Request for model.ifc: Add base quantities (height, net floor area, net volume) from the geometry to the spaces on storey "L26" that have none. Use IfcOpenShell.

First a look at what the model holds.

```python
import ifcopenshell
import ifcopenshell.util.element
import ifcopenshell.util.unit

model = ifcopenshell.open("model.ifc")
print(model.schema)
for unit_type in ("LENGTHUNIT", "AREAUNIT", "VOLUMEUNIT"):
    print(unit_type, ifcopenshell.util.unit.calculate_unit_scale(model, unit_type))
storey = next(s for s in model.by_type("IfcBuildingStorey") if s.Name == "L26")
spaces = [e for e in ifcopenshell.util.element.get_decomposition(storey) if e.is_a("IfcSpace")]
for e in sorted(spaces, key=lambda e: e.id()):
    print(e.id(), e.is_a(), e.Name, list(ifcopenshell.util.element.get_psets(e, qtos_only=True)), sep=" | ")
```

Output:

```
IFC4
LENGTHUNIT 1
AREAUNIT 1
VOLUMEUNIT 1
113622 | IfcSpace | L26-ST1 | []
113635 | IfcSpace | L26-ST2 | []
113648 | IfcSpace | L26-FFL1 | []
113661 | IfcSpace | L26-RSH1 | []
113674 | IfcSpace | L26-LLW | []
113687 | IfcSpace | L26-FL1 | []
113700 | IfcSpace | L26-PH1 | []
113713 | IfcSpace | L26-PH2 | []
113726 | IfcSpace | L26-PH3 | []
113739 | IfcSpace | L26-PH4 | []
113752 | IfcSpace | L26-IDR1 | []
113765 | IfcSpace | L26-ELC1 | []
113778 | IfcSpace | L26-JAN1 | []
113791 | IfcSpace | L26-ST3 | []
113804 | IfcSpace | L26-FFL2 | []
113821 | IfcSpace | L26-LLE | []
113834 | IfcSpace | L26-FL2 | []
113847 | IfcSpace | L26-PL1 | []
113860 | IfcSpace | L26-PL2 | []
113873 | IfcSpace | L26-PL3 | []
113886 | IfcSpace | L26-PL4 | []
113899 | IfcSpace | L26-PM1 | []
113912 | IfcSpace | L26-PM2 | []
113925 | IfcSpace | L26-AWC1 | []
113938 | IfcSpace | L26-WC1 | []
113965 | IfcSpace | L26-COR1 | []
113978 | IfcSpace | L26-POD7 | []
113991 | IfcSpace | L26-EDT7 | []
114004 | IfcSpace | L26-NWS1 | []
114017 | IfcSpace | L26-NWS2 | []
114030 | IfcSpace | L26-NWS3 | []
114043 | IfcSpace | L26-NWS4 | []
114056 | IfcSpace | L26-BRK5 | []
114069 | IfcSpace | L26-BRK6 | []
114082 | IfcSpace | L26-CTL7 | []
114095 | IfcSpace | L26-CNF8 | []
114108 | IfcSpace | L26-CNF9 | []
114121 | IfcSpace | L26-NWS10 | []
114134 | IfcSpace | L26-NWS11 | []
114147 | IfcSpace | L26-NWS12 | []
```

```python
import ifcopenshell
import ifcopenshell.api.pset
import ifcopenshell.geom
import ifcopenshell.util.element
import ifcopenshell.util.shape
import ifcopenshell.util.unit

model = ifcopenshell.open("model.ifc")
unit_scale = ifcopenshell.util.unit.calculate_unit_scale(model)
area_scale = ifcopenshell.util.unit.calculate_unit_scale(model, "AREAUNIT")
volume_scale = ifcopenshell.util.unit.calculate_unit_scale(model, "VOLUMEUNIT")
settings = ifcopenshell.geom.settings()

storey = next(s for s in model.by_type("IfcBuildingStorey") if s.Name == "L26")
spaces = [e for e in ifcopenshell.util.element.get_decomposition(storey) if e.is_a("IfcSpace")]

for e in sorted(spaces, key=lambda e: e.id()):
    if ifcopenshell.util.element.get_psets(e, qtos_only=True, should_inherit=False):
        continue
    # Geometry comes back in metres, in the element's own axes.
    shape = ifcopenshell.geom.create_shape(settings, e)
    values = {
        "Height": ifcopenshell.util.shape.get_z(shape.geometry) / unit_scale,
        "NetFloorArea": ifcopenshell.util.shape.get_footprint_area(shape.geometry) / area_scale,
        "NetVolume": ifcopenshell.util.shape.get_volume(shape.geometry) / volume_scale,
    }
    qto = ifcopenshell.api.pset.add_qto(model, product=e, name="Qto_SpaceBaseQuantities")
    ifcopenshell.api.pset.edit_qto(model, qto=qto, properties=values)
    print(e.id(), {k: round(v, 3) for k, v in values.items()})

model.write("model_rev.ifc")
```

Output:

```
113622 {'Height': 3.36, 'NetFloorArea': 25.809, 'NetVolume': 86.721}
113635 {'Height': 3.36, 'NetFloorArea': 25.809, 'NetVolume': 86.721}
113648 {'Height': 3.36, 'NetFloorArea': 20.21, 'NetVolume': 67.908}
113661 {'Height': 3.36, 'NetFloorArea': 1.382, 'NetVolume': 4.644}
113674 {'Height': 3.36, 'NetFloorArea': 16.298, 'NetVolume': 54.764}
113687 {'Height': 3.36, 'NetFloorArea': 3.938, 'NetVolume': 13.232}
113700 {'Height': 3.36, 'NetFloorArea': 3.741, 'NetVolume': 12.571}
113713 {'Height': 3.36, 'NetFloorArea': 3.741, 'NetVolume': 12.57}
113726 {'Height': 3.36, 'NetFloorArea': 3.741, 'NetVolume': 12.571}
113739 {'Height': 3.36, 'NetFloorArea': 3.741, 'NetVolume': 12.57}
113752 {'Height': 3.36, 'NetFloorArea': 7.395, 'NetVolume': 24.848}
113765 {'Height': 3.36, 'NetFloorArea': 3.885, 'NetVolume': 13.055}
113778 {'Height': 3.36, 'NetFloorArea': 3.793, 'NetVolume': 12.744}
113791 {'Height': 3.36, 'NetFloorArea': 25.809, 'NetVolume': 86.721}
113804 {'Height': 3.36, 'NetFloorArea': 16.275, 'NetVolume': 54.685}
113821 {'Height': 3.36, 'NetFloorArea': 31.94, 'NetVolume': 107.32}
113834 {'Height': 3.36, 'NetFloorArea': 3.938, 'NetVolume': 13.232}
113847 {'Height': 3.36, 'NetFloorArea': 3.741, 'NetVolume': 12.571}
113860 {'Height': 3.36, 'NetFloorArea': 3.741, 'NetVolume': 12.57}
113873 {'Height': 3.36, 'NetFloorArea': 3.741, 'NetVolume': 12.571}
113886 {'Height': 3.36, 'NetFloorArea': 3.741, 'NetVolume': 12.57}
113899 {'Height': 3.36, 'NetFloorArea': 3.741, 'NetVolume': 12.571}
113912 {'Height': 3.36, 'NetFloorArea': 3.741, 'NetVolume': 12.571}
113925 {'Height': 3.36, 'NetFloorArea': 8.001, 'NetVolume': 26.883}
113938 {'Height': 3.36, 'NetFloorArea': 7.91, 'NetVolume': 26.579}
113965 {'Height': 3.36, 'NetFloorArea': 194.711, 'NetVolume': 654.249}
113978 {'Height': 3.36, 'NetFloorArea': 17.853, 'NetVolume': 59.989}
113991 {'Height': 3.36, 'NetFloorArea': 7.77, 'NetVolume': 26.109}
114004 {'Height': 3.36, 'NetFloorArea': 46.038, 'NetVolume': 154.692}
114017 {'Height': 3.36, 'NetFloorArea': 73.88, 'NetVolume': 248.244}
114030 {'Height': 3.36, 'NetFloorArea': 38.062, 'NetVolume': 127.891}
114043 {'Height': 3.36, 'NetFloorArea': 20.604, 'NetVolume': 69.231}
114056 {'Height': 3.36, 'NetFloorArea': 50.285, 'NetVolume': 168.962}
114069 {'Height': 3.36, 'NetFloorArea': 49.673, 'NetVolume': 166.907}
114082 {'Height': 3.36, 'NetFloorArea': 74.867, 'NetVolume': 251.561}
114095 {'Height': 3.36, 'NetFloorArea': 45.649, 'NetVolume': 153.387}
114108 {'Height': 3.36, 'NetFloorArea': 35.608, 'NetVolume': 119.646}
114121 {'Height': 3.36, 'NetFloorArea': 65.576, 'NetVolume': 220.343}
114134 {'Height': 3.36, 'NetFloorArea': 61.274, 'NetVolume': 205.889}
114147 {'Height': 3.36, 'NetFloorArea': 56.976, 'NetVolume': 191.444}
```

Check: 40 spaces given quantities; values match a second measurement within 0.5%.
